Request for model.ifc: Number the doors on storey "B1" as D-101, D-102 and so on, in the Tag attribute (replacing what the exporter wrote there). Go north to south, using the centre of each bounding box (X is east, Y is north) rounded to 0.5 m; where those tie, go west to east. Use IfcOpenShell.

First a look at what the model holds.

```python
import ifcopenshell
import ifcopenshell.util.element
import ifcopenshell.util.placement

model = ifcopenshell.open("model.ifc")
print(model.schema)
storey = next(s for s in model.by_type("IfcBuildingStorey") if s.Name == "B1")
doors = [e for e in ifcopenshell.util.element.get_decomposition(storey) if e.is_a("IfcDoor")]
for e in sorted(doors, key=lambda e: e.id()):
    origin = ifcopenshell.util.placement.get_local_placement(e.ObjectPlacement)[:3, 3]
    print(e.id(), e.Tag, e.Name, origin.round(2) + 0.0, sep=" | ")
```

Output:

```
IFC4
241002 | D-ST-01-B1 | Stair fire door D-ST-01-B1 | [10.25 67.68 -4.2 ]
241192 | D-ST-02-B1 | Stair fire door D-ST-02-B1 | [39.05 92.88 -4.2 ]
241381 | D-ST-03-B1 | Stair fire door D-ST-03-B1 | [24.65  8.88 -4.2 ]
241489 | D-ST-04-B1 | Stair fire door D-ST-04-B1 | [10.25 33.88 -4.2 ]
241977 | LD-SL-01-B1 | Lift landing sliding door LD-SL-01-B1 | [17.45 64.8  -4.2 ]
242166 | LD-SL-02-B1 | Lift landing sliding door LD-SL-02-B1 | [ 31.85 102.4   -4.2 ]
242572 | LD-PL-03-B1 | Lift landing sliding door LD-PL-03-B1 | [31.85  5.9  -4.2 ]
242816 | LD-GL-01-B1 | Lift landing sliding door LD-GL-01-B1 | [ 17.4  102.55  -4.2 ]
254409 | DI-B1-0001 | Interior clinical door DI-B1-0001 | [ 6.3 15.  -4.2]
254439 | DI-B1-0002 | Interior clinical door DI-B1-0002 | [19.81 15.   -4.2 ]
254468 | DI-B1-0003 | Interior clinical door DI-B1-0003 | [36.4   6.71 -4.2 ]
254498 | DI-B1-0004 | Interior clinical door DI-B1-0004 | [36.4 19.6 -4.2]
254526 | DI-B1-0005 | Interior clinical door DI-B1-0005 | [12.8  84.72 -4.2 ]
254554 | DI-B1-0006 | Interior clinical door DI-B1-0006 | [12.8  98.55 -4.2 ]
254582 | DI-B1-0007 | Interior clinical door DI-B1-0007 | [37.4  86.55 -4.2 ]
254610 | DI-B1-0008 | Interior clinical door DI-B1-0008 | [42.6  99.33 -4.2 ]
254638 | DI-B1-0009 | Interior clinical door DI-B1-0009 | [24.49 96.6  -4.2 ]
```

```python
import ifcopenshell
import ifcopenshell.geom
import ifcopenshell.util.element
import ifcopenshell.util.shape

model = ifcopenshell.open("model.ifc")
settings = ifcopenshell.geom.settings()
settings.set("use-world-coords", True)


def centre(element):
    shape = ifcopenshell.geom.create_shape(settings, element)
    return ifcopenshell.util.shape.get_bbox_centroid(shape.geometry)


storey = next(s for s in model.by_type("IfcBuildingStorey") if s.Name == "B1")
doors = [e for e in ifcopenshell.util.element.get_decomposition(storey) if e.is_a("IfcDoor")]

# Insertion points can sit at a corner or the storey origin, so sort by the geometry (in metres).
centres = {e: centre(e) for e in doors}
doors.sort(key=lambda e: (-round(centres[e][1] / 0.5), centres[e][0]))

for i, e in enumerate(doors, start=1):
    number = f"D-1{i:02d}"
    e.Tag = number
    print(e.id(), number)

model.write("model-out.ifc")
```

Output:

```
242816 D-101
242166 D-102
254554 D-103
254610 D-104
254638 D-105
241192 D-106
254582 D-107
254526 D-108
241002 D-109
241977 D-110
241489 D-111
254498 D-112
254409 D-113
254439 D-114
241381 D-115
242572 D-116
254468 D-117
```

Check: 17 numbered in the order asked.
